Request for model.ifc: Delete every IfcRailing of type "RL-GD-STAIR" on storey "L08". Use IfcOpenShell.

First a look at what the model holds.

```python
import ifcopenshell
import ifcopenshell.util.element

model = ifcopenshell.open("model.ifc")
print(model.schema)
storey = next(s for s in model.by_type("IfcBuildingStorey") if s.Name == "L08")
railings = [e for e in ifcopenshell.util.element.get_decomposition(storey) if e.is_a("IfcRailing")]
seen = {}
for e in railings:
    element_type = ifcopenshell.util.element.get_type(e)
    name = element_type.Name if element_type not in (None, e) else None
    seen[name] = seen.get(name, 0) + 1
for name, count in sorted(seen.items(), key=str):
    print(count, "x", name)
```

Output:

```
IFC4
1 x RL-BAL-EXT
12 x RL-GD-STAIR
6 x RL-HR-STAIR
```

```python
import ifcopenshell
import ifcopenshell.api.root
import ifcopenshell.util.element

model = ifcopenshell.open("model.ifc")

storey = next(s for s in model.by_type("IfcBuildingStorey") if s.Name == "L08")
railings = [e for e in ifcopenshell.util.element.get_decomposition(storey) if e.is_a("IfcRailing")]
targets = [e for e in railings if (t := ifcopenshell.util.element.get_type(e)) not in (None, e) and t.Name == "RL-GD-STAIR"]

for e in targets:
    ifcopenshell.api.root.remove_product(model, product=e)
print(len(targets), "removed")

model.write("model_updated.ifc")
```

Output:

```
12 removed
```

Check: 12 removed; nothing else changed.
